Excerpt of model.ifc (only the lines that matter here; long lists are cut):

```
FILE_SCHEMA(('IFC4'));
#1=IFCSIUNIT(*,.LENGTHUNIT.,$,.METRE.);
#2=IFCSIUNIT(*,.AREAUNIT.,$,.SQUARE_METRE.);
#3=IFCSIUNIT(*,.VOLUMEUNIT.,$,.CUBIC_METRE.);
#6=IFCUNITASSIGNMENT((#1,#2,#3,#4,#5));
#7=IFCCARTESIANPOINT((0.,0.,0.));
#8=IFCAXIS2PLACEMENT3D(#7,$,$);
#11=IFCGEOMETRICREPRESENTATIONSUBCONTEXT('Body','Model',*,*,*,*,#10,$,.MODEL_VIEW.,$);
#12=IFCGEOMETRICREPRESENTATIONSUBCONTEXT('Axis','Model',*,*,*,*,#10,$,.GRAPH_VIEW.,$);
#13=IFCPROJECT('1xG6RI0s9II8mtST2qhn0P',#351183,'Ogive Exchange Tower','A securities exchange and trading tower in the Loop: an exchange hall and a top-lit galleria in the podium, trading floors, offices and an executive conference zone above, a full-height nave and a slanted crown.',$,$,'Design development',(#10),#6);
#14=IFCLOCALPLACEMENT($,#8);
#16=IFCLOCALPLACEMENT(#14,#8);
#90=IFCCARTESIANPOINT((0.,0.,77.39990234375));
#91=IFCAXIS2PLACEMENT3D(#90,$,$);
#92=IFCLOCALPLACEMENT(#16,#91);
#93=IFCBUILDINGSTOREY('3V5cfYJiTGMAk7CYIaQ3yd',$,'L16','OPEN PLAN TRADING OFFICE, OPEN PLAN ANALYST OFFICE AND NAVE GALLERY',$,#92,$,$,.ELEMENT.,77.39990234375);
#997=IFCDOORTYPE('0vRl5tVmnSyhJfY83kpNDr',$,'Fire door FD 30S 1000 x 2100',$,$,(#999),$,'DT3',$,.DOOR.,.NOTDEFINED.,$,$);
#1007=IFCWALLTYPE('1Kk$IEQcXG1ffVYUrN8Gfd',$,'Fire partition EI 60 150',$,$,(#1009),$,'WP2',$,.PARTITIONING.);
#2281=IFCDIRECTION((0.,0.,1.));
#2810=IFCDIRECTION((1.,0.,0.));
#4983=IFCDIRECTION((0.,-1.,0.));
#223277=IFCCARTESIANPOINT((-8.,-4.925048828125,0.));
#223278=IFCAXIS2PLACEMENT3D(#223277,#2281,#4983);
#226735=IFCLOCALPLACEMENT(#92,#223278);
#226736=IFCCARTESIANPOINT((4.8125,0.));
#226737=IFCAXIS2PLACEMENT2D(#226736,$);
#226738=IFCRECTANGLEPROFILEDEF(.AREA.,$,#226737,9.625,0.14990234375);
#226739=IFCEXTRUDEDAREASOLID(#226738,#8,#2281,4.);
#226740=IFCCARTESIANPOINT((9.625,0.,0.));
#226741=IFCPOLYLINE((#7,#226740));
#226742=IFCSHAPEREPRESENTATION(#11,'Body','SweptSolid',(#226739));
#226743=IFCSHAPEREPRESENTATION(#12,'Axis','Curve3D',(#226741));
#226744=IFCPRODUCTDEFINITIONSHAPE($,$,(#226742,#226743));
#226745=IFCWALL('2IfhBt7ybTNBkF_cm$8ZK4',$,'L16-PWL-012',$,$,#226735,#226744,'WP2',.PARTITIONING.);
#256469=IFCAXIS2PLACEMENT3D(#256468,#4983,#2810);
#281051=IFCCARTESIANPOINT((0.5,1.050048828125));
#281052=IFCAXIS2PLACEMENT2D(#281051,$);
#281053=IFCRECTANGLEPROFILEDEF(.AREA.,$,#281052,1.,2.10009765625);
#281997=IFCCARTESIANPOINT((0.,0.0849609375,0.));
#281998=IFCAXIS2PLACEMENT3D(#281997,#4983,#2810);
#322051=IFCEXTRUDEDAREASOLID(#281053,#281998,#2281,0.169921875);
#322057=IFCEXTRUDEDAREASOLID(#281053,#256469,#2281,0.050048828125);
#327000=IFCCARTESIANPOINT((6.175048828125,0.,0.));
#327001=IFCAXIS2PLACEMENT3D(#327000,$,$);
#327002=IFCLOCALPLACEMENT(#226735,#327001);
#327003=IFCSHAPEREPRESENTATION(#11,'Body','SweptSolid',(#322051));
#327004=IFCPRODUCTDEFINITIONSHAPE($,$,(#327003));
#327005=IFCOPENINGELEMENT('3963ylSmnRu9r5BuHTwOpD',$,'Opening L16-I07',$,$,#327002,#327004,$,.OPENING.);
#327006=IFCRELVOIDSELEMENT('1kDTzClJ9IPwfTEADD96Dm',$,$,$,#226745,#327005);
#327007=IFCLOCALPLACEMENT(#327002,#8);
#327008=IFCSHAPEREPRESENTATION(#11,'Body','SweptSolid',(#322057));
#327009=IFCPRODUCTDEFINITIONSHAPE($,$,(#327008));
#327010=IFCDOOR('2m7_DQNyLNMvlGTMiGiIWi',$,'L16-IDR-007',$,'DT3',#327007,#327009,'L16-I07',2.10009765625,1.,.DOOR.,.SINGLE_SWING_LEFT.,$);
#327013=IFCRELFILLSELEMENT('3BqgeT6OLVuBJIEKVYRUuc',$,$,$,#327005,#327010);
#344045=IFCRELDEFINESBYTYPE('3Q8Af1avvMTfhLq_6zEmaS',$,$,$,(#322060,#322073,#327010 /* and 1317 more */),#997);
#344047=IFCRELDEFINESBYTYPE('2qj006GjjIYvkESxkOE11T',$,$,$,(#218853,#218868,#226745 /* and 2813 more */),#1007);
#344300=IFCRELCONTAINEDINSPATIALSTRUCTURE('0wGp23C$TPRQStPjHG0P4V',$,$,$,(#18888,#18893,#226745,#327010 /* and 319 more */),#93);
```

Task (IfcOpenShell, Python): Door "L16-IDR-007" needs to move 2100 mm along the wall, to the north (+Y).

```python
import ifcopenshell
import ifcopenshell.api.geometry
import ifcopenshell.util.placement
import ifcopenshell.util.unit

model = ifcopenshell.open("model.ifc")
unit_scale = ifcopenshell.util.unit.calculate_unit_scale(model)

door = model.by_guid("2m7_DQNyLNMvlGTMiGiIWi")
opening = door.FillsVoids[0].RelatingOpeningElement
wall = opening.VoidsElements[0].RelatingBuildingElement

wall_matrix = ifcopenshell.util.placement.get_local_placement(wall.ObjectPlacement)
shift = wall_matrix[:3, 0] * -2.1 / unit_scale
before = ifcopenshell.util.placement.get_local_placement(door.ObjectPlacement)[:3, 3].copy()

# The door is placed relative to its opening, so it follows when the opening moves.
matrix = ifcopenshell.util.placement.get_local_placement(opening.ObjectPlacement)
matrix[:3, 3] += shift
ifcopenshell.api.geometry.edit_object_placement(
    model, product=opening, matrix=matrix, is_si=False, should_transform_children=True
)

after = ifcopenshell.util.placement.get_local_placement(door.ObjectPlacement)[:3, 3]
print("door moved by", (after - before).round(3) + 0.0)

model.write("model_edited.ifc")
```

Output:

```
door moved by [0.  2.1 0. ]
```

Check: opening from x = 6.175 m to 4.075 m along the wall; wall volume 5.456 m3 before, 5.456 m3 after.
